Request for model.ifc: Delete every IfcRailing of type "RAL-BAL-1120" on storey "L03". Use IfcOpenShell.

First a look at what the model holds.

```python
import ifcopenshell
import ifcopenshell.util.element

model = ifcopenshell.open("model.ifc")
print(model.schema)
storey = next(s for s in model.by_type("IfcBuildingStorey") if s.Name == "L03")
railings = [e for e in ifcopenshell.util.element.get_decomposition(storey) if e.is_a("IfcRailing")]
seen = {}
for e in railings:
    element_type = ifcopenshell.util.element.get_type(e)
    name = element_type.Name if element_type not in (None, e) else None
    seen[name] = seen.get(name, 0) + 1
for name, count in sorted(seen.items(), key=str):
    print(count, "x", name)
```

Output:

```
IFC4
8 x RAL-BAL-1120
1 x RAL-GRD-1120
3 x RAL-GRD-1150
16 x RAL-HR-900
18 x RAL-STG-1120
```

```python
import ifcopenshell
import ifcopenshell.api.root
import ifcopenshell.util.element

model = ifcopenshell.open("model.ifc")

storey = next(s for s in model.by_type("IfcBuildingStorey") if s.Name == "L03")
railings = [e for e in ifcopenshell.util.element.get_decomposition(storey) if e.is_a("IfcRailing")]
targets = [e for e in railings if (t := ifcopenshell.util.element.get_type(e)) not in (None, e) and t.Name == "RAL-BAL-1120"]

for e in targets:
    ifcopenshell.api.root.remove_product(model, product=e)
print(len(targets), "removed")

model.write("model_updated.ifc")
```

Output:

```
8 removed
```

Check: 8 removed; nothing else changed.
